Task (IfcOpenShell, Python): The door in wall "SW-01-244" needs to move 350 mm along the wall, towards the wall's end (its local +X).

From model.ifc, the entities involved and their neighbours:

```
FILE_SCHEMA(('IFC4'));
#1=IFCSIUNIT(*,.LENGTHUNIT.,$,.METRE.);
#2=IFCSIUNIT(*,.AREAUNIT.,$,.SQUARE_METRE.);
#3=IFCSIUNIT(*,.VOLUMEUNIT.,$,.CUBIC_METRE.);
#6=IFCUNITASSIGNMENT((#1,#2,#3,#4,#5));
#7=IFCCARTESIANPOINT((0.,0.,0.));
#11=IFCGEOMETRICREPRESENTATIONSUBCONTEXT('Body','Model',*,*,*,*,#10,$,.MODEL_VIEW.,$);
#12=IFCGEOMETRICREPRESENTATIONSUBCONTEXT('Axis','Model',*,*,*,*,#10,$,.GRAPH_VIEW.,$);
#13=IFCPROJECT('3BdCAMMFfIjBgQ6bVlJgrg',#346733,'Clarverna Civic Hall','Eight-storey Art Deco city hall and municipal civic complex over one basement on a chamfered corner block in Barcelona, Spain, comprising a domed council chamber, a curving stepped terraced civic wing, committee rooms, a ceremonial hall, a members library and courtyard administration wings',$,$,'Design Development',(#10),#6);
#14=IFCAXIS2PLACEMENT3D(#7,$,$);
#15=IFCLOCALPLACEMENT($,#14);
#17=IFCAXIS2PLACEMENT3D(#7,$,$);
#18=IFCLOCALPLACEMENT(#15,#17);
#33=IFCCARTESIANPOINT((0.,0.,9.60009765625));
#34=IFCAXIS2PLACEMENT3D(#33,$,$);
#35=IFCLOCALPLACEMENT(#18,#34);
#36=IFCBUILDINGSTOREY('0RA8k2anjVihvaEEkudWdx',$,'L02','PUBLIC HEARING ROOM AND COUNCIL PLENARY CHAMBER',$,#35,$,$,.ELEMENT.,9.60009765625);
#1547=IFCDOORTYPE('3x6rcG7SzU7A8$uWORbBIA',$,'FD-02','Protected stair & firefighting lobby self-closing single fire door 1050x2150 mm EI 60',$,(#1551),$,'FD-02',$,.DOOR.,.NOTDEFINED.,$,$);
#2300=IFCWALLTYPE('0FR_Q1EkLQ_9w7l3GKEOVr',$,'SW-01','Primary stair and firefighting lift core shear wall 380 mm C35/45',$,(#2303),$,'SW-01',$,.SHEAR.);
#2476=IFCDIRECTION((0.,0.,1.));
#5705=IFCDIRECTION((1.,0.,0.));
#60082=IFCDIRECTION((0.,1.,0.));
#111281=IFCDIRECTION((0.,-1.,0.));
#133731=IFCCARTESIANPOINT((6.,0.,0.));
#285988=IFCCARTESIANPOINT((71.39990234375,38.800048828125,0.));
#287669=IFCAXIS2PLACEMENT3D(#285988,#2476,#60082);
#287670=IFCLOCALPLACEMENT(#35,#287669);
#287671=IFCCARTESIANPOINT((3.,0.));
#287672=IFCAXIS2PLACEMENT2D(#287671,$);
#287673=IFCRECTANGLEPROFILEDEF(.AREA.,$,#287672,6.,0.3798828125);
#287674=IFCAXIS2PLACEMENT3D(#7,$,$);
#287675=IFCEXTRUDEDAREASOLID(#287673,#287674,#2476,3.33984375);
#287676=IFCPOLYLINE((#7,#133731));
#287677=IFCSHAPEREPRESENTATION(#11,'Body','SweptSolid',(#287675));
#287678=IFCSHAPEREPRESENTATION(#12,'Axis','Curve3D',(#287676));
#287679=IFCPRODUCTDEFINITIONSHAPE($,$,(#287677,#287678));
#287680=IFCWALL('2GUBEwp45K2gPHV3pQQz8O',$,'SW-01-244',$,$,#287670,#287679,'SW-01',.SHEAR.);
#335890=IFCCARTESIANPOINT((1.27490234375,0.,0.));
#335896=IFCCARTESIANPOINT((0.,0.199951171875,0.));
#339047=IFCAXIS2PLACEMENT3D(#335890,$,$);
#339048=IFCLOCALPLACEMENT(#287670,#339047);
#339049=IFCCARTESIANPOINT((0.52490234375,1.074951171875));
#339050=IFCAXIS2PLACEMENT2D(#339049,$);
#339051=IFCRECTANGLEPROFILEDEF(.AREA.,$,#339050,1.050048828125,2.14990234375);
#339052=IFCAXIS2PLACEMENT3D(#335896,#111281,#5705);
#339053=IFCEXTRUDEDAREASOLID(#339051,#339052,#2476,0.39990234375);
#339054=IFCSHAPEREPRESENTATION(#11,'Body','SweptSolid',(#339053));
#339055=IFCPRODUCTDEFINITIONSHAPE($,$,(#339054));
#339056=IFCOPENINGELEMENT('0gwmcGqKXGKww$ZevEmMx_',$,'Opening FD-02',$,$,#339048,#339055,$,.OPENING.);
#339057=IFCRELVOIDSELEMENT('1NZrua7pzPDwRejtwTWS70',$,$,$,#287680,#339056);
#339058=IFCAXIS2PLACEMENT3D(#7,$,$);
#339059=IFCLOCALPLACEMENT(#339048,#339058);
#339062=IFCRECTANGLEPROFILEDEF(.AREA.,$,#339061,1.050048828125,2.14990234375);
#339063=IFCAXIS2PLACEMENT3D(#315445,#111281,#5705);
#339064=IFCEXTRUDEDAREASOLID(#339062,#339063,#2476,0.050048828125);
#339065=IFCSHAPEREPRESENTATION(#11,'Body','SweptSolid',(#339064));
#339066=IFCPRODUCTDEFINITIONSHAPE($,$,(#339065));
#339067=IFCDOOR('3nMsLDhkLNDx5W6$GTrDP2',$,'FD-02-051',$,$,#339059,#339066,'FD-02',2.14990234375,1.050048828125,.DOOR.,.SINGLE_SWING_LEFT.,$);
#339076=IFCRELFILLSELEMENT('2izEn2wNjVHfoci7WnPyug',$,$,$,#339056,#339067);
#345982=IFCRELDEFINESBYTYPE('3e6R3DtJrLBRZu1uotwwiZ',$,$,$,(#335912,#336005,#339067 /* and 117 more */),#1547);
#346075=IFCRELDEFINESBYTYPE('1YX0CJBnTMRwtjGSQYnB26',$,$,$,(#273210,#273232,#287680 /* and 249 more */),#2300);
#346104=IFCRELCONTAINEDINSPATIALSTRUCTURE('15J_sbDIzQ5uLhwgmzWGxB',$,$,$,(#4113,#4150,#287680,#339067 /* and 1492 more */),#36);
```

```python
import ifcopenshell
import ifcopenshell.api.geometry
import ifcopenshell.util.placement

model = ifcopenshell.open("model.ifc")

door = model.by_guid("3nMsLDhkLNDx5W6$GTrDP2")
opening = door.FillsVoids[0].RelatingOpeningElement
wall = opening.VoidsElements[0].RelatingBuildingElement

wall_matrix = ifcopenshell.util.placement.get_local_placement(wall.ObjectPlacement)
shift = wall_matrix[:3, 0] * 0.35
before = ifcopenshell.util.placement.get_local_placement(door.ObjectPlacement)[:3, 3].copy()

# The door is placed relative to its opening, so it follows when the opening moves.
matrix = ifcopenshell.util.placement.get_local_placement(opening.ObjectPlacement)
matrix[:3, 3] += shift
ifcopenshell.api.geometry.edit_object_placement(
    model, product=opening, matrix=matrix, is_si=False, should_transform_children=True
)

after = ifcopenshell.util.placement.get_local_placement(door.ObjectPlacement)[:3, 3]
print("door moved by", (after - before).round(3) + 0.0)

model.write("model_v2.ifc")
```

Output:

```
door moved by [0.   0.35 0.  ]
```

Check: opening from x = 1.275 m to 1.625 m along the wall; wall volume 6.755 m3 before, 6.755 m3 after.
